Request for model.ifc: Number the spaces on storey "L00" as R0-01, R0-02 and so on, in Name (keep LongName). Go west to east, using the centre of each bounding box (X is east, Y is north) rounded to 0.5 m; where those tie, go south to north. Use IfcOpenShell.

First a look at what the model holds.

```python
import ifcopenshell
import ifcopenshell.util.element
import ifcopenshell.util.placement

model = ifcopenshell.open("model.ifc")
print(model.schema)
storey = next(s for s in model.by_type("IfcBuildingStorey") if s.Name == "L00")
spaces = [e for e in ifcopenshell.util.element.get_decomposition(storey) if e.is_a("IfcSpace")]
for e in sorted(spaces, key=lambda e: e.id()):
    origin = ifcopenshell.util.placement.get_local_placement(e.ObjectPlacement)[:3, 3]
    print(e.id(), e.Name, e.LongName, origin.round(2) + 0.0, sep=" | ")
```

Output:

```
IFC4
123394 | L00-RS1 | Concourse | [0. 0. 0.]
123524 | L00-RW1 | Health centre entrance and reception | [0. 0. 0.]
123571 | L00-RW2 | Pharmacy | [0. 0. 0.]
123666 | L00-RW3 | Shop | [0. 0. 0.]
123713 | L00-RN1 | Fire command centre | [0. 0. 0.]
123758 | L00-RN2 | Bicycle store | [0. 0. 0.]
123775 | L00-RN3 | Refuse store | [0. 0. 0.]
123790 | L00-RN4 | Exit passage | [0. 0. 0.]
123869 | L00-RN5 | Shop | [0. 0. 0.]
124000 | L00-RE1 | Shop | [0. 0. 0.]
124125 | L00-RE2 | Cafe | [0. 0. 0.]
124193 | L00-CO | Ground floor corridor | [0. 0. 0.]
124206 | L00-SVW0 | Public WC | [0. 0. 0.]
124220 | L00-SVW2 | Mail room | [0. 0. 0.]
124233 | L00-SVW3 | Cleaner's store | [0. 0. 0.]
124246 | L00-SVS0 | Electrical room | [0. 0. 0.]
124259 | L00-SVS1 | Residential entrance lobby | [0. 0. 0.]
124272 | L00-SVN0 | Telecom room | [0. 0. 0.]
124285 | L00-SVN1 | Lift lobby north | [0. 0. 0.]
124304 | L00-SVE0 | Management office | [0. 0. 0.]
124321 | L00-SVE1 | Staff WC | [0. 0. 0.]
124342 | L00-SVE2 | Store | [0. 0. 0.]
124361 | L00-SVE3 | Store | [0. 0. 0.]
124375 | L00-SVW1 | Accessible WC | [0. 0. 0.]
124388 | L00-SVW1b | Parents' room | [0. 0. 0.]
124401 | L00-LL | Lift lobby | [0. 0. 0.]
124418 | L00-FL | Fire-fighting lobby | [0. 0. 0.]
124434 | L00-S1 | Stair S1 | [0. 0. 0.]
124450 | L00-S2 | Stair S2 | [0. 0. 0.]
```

```python
import ifcopenshell
import ifcopenshell.geom
import ifcopenshell.util.element
import ifcopenshell.util.shape

model = ifcopenshell.open("model.ifc")
settings = ifcopenshell.geom.settings()
settings.set("use-world-coords", True)


def centre(element):
    shape = ifcopenshell.geom.create_shape(settings, element)
    return ifcopenshell.util.shape.get_bbox_centroid(shape.geometry)


storey = next(s for s in model.by_type("IfcBuildingStorey") if s.Name == "L00")
spaces = [e for e in ifcopenshell.util.element.get_decomposition(storey) if e.is_a("IfcSpace")]

# Insertion points can sit at a corner or the storey origin, so sort by the geometry (in metres).
centres = {e: centre(e) for e in spaces}
spaces.sort(key=lambda e: (round(centres[e][0] / 0.5), centres[e][1]))

for i, e in enumerate(spaces, start=1):
    number = f"R0-{i:02d}"
    e.Name = number
    print(e.id(), number)

model.write("model_edited.ifc")
```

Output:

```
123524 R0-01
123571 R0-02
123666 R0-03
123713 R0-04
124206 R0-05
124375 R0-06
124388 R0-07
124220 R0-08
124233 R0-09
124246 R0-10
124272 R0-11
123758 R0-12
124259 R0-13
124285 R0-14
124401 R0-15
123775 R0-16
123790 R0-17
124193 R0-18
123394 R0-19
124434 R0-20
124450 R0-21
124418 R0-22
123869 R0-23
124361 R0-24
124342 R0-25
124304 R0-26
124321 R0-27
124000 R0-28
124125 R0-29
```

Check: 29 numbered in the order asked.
